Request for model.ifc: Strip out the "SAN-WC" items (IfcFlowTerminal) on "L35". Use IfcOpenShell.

First a look at what the model holds.

```python
import ifcopenshell
import ifcopenshell.util.element

model = ifcopenshell.open("model.ifc")
print(model.schema)
storey = next(s for s in model.by_type("IfcBuildingStorey") if s.Name == "L35")
terminals = [e for e in ifcopenshell.util.element.get_decomposition(storey) if e.is_a("IfcFlowTerminal")]
seen = {}
for e in terminals:
    element_type = ifcopenshell.util.element.get_type(e)
    name = element_type.Name if element_type not in (None, e) else None
    seen[name] = seen.get(name, 0) + 1
for name, count in sorted(seen.items(), key=str):
    print(count, "x", name)
```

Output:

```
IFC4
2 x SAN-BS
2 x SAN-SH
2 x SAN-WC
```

```python
import ifcopenshell
import ifcopenshell.api.root
import ifcopenshell.util.element

model = ifcopenshell.open("model.ifc")

storey = next(s for s in model.by_type("IfcBuildingStorey") if s.Name == "L35")
terminals = [e for e in ifcopenshell.util.element.get_decomposition(storey) if e.is_a("IfcFlowTerminal")]
targets = [e for e in terminals if (t := ifcopenshell.util.element.get_type(e)) not in (None, e) and t.Name == "SAN-WC"]

for e in targets:
    ifcopenshell.api.root.remove_product(model, product=e)
print(len(targets), "removed")

model.write("model_updated.ifc")
```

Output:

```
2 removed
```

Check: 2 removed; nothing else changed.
